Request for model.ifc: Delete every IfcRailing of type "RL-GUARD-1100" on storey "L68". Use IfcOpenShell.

First a look at what the model holds.

```python
import ifcopenshell
import ifcopenshell.util.element

model = ifcopenshell.open("model.ifc")
print(model.schema)
storey = next(s for s in model.by_type("IfcBuildingStorey") if s.Name == "L68")
railings = [e for e in ifcopenshell.util.element.get_decomposition(storey) if e.is_a("IfcRailing")]
seen = {}
for e in railings:
    element_type = ifcopenshell.util.element.get_type(e)
    name = element_type.Name if element_type not in (None, e) else None
    seen[name] = seen.get(name, 0) + 1
for name, count in sorted(seen.items(), key=str):
    print(count, "x", name)
```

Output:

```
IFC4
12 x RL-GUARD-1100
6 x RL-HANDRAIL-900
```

```python
import ifcopenshell
import ifcopenshell.api.root
import ifcopenshell.util.element

model = ifcopenshell.open("model.ifc")

storey = next(s for s in model.by_type("IfcBuildingStorey") if s.Name == "L68")
railings = [e for e in ifcopenshell.util.element.get_decomposition(storey) if e.is_a("IfcRailing")]
targets = [e for e in railings if (t := ifcopenshell.util.element.get_type(e)) not in (None, e) and t.Name == "RL-GUARD-1100"]

for e in targets:
    ifcopenshell.api.root.remove_product(model, product=e)
print(len(targets), "removed")

model.write("model_rev.ifc")
```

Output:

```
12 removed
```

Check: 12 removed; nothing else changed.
